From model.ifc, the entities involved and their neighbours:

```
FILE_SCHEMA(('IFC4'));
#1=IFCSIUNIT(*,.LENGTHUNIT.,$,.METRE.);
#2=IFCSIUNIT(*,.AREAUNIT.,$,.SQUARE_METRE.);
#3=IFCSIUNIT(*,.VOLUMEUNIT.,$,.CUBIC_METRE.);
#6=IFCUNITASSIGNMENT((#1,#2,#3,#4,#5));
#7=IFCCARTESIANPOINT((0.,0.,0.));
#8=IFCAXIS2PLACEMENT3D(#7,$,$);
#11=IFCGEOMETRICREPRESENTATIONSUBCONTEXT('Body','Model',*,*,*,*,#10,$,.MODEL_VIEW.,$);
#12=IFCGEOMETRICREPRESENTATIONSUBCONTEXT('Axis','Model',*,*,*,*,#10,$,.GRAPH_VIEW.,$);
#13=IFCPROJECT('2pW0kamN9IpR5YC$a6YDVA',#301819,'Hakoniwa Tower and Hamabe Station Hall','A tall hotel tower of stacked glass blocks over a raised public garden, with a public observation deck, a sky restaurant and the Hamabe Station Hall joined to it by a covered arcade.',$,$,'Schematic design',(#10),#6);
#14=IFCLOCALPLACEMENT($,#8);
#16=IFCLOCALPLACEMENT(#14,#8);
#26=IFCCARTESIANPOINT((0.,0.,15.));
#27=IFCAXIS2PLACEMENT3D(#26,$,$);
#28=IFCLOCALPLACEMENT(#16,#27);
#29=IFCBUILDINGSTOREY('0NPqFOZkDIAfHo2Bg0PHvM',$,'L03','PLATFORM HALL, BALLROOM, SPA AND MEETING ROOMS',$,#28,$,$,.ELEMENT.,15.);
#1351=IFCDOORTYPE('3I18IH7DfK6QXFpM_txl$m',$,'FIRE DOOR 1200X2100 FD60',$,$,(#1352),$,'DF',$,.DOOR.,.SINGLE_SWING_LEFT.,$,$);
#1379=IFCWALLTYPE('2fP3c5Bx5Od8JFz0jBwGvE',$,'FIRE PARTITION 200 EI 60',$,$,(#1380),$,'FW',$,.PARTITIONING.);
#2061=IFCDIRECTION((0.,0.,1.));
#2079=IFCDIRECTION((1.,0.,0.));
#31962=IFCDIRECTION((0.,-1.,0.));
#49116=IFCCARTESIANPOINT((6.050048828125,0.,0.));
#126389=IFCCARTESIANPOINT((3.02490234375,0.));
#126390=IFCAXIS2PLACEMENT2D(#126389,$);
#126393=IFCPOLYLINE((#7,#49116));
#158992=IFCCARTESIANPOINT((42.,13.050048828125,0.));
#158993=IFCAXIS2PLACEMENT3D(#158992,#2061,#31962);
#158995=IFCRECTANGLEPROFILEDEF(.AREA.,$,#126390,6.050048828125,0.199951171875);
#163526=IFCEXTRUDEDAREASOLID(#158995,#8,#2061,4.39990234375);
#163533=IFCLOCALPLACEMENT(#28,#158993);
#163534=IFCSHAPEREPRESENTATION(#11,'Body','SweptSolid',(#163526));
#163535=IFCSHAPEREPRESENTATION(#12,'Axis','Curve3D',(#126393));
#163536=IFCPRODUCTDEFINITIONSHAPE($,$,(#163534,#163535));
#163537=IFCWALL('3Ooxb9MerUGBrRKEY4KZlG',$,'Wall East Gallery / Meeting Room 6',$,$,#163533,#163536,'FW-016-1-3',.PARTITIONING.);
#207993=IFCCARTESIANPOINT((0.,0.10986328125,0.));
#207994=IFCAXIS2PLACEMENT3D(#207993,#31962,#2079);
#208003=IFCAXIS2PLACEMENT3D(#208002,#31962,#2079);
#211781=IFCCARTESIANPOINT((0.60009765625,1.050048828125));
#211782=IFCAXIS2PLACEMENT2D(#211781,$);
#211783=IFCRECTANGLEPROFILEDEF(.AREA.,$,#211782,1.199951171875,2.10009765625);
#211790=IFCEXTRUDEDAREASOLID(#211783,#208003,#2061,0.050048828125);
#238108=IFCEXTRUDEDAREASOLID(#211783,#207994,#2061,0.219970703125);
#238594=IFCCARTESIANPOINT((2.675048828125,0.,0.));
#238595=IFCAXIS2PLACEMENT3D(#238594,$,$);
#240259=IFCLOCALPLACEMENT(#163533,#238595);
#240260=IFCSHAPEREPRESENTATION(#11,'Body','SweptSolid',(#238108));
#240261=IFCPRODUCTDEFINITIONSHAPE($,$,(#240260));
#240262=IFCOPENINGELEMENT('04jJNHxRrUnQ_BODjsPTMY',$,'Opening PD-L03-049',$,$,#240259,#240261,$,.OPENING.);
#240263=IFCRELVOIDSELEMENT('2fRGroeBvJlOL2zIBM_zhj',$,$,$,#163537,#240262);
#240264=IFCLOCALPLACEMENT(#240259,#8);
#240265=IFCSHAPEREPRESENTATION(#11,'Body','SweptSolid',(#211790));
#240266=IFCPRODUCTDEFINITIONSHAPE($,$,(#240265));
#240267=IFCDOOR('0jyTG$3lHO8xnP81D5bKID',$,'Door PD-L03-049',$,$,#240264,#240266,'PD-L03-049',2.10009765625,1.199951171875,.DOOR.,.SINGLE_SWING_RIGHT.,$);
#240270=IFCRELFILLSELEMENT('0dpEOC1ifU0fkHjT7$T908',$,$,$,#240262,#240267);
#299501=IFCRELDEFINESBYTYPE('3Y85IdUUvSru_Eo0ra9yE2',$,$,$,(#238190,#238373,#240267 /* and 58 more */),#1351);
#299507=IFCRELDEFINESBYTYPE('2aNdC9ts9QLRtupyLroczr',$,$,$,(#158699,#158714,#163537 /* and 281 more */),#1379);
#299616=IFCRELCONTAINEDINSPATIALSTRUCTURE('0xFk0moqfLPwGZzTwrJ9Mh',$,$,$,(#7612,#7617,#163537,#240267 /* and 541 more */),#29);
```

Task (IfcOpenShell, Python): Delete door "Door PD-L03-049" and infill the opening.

```python
import ifcopenshell
import ifcopenshell.api.feature
import ifcopenshell.api.root
import ifcopenshell.geom
import ifcopenshell.util.shape

model = ifcopenshell.open("model.ifc")
settings = ifcopenshell.geom.settings()


def volume(element):
    """Net volume in cubic metres, openings subtracted."""
    shape = ifcopenshell.geom.create_shape(settings, element)
    return ifcopenshell.util.shape.get_volume(shape.geometry)


door = model.by_guid("0jyTG$3lHO8xnP81D5bKID")
opening = door.FillsVoids[0].RelatingOpeningElement
wall = opening.VoidsElements[0].RelatingBuildingElement
before = volume(wall)

ifcopenshell.api.root.remove_product(model, product=door)
ifcopenshell.api.feature.remove_feature(model, feature=opening)

after = volume(wall)

print(f"wall volume {before:.3f} -> {after:.3f} m3")

model.write("model_edited.ifc")
```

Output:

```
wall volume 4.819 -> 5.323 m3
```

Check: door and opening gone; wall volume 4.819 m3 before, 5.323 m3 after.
